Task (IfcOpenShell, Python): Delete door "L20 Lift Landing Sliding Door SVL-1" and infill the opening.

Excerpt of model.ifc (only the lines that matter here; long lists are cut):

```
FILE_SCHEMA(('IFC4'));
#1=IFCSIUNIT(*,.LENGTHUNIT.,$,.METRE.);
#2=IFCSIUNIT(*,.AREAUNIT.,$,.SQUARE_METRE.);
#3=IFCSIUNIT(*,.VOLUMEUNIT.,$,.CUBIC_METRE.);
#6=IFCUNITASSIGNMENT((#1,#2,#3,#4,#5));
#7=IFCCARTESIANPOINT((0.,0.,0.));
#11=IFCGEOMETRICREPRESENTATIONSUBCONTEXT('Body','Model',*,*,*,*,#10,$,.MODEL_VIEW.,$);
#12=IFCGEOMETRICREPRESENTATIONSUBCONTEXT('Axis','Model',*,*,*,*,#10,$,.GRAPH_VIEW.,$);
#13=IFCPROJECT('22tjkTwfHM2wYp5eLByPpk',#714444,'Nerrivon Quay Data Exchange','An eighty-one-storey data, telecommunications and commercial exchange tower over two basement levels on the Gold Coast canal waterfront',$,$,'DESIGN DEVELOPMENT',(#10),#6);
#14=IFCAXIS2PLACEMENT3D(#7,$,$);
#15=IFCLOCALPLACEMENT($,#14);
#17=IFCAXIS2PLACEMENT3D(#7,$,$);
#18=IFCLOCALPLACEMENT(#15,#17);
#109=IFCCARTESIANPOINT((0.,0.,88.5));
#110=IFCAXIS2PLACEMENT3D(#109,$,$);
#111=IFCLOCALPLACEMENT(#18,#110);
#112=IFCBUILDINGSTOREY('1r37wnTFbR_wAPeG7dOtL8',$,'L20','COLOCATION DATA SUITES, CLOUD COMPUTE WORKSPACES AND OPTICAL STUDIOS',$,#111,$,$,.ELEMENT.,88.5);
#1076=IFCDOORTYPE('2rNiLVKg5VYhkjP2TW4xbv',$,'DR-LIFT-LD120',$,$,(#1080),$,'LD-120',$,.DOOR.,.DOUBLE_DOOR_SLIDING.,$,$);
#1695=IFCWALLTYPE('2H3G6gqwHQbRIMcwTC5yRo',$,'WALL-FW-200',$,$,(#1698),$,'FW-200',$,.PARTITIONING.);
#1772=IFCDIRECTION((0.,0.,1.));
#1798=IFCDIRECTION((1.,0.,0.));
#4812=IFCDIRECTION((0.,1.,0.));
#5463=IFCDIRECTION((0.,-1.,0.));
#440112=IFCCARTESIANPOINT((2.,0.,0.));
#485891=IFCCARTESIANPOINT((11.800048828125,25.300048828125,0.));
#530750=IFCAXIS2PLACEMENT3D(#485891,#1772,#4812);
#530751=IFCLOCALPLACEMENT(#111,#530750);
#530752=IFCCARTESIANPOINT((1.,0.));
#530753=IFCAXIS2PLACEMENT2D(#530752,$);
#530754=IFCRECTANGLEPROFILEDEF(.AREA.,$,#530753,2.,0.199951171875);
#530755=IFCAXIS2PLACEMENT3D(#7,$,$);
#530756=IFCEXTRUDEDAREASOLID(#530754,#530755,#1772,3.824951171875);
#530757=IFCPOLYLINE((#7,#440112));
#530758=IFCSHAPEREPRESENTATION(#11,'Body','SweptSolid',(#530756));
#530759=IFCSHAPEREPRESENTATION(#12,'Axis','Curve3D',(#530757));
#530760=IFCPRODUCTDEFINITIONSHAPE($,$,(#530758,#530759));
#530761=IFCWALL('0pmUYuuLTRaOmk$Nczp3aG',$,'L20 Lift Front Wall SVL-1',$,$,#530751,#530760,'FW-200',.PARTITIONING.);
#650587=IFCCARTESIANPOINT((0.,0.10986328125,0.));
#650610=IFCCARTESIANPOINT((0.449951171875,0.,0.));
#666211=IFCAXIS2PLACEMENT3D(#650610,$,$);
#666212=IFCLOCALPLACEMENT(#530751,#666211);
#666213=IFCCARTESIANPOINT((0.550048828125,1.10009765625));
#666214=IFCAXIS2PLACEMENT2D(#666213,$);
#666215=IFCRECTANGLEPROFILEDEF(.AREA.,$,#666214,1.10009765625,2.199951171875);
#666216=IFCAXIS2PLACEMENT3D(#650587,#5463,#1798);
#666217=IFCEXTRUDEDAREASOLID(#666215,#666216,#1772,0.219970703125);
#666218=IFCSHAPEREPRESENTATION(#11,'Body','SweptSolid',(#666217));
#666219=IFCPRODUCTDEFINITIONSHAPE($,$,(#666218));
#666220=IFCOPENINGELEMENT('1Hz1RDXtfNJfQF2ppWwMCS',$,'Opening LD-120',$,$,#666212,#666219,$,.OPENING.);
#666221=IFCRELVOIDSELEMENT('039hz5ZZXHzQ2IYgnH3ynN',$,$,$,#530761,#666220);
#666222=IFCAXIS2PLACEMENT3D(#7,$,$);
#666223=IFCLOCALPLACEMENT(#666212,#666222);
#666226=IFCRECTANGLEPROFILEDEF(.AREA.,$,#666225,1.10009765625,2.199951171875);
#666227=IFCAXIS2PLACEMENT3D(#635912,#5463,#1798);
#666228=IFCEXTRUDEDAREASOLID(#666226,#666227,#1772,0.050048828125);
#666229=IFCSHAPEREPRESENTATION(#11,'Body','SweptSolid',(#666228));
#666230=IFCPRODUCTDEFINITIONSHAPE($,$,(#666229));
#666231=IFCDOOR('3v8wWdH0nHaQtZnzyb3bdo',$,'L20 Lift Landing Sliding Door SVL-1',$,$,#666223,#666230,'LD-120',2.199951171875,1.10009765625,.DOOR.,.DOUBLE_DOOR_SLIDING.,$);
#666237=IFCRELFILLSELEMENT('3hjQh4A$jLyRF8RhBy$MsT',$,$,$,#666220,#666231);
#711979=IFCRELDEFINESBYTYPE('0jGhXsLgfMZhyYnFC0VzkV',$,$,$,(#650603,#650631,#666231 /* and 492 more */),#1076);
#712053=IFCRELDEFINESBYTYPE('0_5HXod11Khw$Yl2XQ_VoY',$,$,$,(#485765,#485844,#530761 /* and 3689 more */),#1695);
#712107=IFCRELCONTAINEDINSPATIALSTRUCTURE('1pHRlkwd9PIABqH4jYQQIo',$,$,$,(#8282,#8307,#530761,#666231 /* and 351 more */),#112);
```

```python
import ifcopenshell
import ifcopenshell.api.feature
import ifcopenshell.api.root
import ifcopenshell.geom
import ifcopenshell.util.shape

model = ifcopenshell.open("model.ifc")
settings = ifcopenshell.geom.settings()


def volume(element):
    """Net volume in cubic metres, openings subtracted."""
    shape = ifcopenshell.geom.create_shape(settings, element)
    return ifcopenshell.util.shape.get_volume(shape.geometry)


door = model.by_guid("3v8wWdH0nHaQtZnzyb3bdo")
opening = door.FillsVoids[0].RelatingOpeningElement
wall = opening.VoidsElements[0].RelatingBuildingElement
before = volume(wall)

ifcopenshell.api.root.remove_product(model, product=door)
ifcopenshell.api.feature.remove_feature(model, feature=opening)

after = volume(wall)

print(f"wall volume {before:.3f} -> {after:.3f} m3")

model.write("model_edited.ifc")
```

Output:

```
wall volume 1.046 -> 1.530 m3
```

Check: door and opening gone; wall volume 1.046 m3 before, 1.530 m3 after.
